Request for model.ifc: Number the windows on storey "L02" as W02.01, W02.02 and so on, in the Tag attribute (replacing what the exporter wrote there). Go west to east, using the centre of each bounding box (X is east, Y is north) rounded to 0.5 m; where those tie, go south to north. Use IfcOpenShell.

First a look at what the model holds.

```python
import ifcopenshell
import ifcopenshell.util.element
import ifcopenshell.util.placement

model = ifcopenshell.open("model.ifc")
print(model.schema)
storey = next(s for s in model.by_type("IfcBuildingStorey") if s.Name == "L02")
windows = [e for e in ifcopenshell.util.element.get_decomposition(storey) if e.is_a("IfcWindow")]
for e in sorted(windows, key=lambda e: e.id()):
    origin = ifcopenshell.util.placement.get_local_placement(e.ObjectPlacement)[:3, 3]
    print(e.id(), e.Tag, e.Name, origin.round(2) + 0.0, sep=" | ")
```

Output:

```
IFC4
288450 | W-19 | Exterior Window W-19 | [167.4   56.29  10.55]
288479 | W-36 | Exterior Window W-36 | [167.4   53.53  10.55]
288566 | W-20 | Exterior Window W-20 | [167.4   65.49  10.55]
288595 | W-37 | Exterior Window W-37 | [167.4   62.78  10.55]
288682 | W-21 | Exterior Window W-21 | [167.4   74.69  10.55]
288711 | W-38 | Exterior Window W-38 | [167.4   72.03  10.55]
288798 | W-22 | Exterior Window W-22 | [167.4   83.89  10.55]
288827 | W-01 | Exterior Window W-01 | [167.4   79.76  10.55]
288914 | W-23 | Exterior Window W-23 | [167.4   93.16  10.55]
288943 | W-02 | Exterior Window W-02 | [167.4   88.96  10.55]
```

```python
import ifcopenshell
import ifcopenshell.geom
import ifcopenshell.util.element
import ifcopenshell.util.shape

model = ifcopenshell.open("model.ifc")
settings = ifcopenshell.geom.settings()
settings.set("use-world-coords", True)


def centre(element):
    shape = ifcopenshell.geom.create_shape(settings, element)
    return ifcopenshell.util.shape.get_bbox_centroid(shape.geometry)


storey = next(s for s in model.by_type("IfcBuildingStorey") if s.Name == "L02")
windows = [e for e in ifcopenshell.util.element.get_decomposition(storey) if e.is_a("IfcWindow")]

# Insertion points can sit at a corner or the storey origin, so sort by the geometry (in metres).
centres = {e: centre(e) for e in windows}
windows.sort(key=lambda e: (round(centres[e][0] / 0.5), centres[e][1]))

for i, e in enumerate(windows, start=1):
    number = f"W02.{i:02d}"
    e.Tag = number
    print(e.id(), number)

model.write("model_updated.ifc")
```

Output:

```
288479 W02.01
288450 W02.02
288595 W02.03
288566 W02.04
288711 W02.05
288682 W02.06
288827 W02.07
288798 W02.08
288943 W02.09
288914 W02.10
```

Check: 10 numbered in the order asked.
